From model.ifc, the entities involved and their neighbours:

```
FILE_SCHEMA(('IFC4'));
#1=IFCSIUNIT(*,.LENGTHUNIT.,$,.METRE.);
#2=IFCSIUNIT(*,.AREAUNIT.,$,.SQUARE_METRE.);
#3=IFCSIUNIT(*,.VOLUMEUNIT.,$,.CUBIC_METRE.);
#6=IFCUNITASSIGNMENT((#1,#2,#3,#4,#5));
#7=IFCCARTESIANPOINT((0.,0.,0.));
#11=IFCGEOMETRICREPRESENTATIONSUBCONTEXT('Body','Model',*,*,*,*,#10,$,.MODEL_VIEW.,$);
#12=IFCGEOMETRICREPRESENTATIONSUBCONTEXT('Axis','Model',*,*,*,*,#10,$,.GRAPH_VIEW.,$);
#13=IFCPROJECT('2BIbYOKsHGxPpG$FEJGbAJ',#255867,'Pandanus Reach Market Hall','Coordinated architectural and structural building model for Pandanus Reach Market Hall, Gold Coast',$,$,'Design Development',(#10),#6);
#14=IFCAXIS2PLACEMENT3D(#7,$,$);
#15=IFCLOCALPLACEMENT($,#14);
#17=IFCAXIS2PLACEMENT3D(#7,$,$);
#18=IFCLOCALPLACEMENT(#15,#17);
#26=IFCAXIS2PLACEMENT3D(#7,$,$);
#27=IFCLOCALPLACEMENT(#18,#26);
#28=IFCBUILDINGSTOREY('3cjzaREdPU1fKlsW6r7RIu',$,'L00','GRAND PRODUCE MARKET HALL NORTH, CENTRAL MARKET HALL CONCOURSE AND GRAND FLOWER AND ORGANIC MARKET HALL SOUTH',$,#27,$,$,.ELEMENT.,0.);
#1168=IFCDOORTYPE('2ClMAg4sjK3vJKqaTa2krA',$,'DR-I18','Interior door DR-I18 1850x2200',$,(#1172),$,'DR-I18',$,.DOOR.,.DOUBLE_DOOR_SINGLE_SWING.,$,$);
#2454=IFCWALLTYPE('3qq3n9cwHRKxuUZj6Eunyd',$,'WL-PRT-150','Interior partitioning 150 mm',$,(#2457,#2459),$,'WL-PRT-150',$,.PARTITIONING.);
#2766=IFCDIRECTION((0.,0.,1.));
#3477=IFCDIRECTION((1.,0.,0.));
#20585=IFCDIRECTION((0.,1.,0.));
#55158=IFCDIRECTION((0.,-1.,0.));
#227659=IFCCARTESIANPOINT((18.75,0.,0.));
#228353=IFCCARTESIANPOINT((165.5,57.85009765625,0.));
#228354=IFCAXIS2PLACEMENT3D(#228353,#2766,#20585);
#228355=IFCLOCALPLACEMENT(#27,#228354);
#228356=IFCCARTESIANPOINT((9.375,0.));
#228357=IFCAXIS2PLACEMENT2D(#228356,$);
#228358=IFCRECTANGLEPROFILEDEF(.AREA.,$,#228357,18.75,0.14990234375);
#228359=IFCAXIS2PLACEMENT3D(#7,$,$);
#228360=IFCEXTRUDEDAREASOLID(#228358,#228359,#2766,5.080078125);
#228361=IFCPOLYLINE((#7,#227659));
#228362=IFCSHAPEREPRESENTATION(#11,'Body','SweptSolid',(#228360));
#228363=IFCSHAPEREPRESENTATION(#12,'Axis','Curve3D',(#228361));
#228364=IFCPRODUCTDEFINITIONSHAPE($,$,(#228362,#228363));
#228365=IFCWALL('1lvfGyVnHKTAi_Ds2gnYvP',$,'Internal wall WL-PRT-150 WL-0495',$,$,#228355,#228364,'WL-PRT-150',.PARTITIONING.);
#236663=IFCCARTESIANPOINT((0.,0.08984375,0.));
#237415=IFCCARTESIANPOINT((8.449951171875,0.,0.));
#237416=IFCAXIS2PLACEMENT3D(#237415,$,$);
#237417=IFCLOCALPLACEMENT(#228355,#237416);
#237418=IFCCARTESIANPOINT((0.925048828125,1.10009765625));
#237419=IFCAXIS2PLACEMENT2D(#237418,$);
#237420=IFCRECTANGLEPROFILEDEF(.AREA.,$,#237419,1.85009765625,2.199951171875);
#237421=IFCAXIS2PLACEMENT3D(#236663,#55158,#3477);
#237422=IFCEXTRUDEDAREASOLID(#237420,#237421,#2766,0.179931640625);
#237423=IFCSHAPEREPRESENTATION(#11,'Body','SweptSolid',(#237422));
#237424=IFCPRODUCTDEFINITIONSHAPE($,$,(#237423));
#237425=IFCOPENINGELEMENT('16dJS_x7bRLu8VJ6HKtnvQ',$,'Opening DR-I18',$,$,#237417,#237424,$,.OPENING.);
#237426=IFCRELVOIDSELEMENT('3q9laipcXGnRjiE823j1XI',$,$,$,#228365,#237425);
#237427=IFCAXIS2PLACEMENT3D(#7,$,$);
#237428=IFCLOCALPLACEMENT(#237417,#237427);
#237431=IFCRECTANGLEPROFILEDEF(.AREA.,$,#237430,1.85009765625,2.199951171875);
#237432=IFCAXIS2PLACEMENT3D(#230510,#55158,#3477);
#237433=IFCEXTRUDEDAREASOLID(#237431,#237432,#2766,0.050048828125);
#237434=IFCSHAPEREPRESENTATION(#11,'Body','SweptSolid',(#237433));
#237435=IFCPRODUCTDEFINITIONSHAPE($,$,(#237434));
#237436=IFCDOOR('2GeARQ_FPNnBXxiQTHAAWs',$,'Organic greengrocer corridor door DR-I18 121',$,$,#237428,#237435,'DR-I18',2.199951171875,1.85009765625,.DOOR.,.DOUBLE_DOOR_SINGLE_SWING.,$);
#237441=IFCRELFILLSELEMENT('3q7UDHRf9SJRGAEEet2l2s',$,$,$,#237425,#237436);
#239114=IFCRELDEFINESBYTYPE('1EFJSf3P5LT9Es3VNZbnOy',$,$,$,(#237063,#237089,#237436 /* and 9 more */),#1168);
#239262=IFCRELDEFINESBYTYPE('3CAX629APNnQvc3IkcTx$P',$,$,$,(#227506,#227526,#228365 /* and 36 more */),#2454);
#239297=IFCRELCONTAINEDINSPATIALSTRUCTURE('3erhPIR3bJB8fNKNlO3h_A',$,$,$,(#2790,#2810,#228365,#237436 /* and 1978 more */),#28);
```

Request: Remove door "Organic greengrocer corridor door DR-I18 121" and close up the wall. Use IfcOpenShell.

```python
import ifcopenshell
import ifcopenshell.api.feature
import ifcopenshell.api.root
import ifcopenshell.geom
import ifcopenshell.util.shape

model = ifcopenshell.open("model.ifc")
settings = ifcopenshell.geom.settings()


def volume(element):
    """Net volume in cubic metres, openings subtracted."""
    shape = ifcopenshell.geom.create_shape(settings, element)
    return ifcopenshell.util.shape.get_volume(shape.geometry)


door = model.by_guid("2GeARQ_FPNnBXxiQTHAAWs")
opening = door.FillsVoids[0].RelatingOpeningElement
wall = opening.VoidsElements[0].RelatingBuildingElement
before = volume(wall)

ifcopenshell.api.root.remove_product(model, product=door)
ifcopenshell.api.feature.remove_feature(model, feature=opening)

after = volume(wall)

print(f"wall volume {before:.3f} -> {after:.3f} m3")

model.write("model_edited.ifc")
```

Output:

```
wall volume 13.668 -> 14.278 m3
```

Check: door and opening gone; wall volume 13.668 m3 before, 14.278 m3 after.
